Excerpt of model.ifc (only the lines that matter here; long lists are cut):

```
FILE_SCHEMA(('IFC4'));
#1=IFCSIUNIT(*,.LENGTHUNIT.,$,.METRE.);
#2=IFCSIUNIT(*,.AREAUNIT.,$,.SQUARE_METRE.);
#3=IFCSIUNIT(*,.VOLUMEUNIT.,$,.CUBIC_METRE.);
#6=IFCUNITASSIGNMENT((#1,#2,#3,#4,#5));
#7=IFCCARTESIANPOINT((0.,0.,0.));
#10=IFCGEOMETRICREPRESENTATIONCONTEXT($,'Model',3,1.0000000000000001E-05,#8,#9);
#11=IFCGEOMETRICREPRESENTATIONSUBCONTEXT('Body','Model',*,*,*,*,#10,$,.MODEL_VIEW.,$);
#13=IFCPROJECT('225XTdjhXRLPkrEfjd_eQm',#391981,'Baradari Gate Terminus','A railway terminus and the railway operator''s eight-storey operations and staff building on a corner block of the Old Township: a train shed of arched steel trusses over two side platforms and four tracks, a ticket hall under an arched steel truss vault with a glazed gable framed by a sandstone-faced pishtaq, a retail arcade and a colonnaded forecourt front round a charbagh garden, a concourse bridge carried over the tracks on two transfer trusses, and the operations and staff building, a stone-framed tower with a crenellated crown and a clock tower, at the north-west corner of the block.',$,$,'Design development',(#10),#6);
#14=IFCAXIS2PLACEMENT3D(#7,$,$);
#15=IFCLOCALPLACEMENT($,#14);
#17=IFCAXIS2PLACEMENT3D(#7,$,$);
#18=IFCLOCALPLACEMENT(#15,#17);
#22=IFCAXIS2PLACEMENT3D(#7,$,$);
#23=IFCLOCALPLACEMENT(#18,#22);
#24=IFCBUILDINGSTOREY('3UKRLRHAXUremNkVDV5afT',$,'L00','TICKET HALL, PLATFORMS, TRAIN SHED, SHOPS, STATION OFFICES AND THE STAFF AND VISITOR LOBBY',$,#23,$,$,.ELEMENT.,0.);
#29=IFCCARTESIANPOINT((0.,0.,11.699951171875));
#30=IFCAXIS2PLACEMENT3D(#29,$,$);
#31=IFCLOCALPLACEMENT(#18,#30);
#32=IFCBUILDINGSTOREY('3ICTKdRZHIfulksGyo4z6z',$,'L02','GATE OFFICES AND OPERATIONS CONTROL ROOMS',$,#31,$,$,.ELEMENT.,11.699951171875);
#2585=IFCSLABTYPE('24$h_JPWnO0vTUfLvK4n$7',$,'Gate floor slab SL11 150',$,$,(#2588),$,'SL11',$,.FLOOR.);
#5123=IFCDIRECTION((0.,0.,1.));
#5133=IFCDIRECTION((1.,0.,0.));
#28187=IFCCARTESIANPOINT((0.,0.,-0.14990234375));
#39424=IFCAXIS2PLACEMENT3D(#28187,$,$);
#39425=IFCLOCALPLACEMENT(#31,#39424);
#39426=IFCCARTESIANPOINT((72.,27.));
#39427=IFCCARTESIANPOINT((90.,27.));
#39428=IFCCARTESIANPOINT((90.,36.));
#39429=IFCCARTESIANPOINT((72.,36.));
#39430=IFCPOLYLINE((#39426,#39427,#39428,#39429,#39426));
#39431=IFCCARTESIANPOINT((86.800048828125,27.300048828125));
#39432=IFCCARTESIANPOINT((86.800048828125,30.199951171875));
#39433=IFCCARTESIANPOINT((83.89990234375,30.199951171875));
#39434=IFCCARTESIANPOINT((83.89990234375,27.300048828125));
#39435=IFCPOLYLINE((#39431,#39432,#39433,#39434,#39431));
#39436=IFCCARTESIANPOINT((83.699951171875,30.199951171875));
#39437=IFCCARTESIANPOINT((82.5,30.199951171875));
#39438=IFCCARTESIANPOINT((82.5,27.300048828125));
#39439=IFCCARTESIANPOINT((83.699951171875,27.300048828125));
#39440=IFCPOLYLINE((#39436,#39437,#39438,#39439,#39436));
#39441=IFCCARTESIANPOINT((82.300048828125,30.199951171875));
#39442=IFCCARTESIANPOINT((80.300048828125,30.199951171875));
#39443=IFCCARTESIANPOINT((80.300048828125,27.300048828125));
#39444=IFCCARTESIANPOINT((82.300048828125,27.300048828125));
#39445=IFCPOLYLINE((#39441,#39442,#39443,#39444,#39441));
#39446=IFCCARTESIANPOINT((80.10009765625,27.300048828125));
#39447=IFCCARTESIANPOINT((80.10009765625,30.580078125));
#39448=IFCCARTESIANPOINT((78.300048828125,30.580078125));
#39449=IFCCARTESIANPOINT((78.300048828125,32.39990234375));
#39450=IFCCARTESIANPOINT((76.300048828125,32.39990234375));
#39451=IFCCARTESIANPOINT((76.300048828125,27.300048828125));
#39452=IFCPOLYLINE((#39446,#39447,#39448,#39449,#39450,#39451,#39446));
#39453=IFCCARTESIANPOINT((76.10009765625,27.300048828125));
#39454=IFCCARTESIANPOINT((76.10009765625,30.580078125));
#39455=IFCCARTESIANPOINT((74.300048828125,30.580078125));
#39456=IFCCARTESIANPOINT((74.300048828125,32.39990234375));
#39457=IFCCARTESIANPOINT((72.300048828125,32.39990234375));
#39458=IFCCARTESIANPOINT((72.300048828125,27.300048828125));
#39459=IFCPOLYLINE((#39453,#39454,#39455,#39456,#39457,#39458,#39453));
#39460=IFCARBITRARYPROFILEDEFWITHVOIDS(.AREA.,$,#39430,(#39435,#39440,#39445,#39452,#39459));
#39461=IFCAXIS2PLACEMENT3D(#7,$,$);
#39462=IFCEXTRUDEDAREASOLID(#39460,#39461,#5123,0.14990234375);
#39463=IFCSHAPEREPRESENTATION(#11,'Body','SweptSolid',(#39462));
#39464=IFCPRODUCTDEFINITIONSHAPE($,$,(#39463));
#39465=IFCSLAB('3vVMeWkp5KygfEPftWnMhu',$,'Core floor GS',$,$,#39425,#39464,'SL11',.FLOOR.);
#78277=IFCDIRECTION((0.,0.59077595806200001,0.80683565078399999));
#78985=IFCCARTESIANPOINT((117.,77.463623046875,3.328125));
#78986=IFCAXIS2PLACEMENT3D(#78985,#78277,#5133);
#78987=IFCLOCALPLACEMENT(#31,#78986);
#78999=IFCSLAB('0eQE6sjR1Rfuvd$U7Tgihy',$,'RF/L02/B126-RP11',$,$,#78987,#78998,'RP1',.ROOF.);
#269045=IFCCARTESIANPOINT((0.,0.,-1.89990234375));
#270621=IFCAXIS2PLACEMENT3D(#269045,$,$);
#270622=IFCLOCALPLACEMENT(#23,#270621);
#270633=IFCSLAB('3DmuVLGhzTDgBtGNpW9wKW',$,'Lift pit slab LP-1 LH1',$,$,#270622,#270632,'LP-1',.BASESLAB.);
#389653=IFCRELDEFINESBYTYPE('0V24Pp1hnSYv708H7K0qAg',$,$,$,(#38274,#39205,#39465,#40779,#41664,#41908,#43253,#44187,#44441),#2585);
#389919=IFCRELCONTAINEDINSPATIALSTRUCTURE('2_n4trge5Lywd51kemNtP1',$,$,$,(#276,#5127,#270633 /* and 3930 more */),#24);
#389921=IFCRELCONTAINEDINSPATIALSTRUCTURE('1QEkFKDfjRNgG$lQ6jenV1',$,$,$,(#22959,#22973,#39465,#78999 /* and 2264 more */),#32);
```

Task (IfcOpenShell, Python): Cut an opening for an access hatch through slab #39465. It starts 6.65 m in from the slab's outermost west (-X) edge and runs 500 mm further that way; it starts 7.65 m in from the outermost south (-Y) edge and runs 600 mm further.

```python
import numpy as np
import ifcopenshell
import ifcopenshell.api.feature
import ifcopenshell.api.geometry
import ifcopenshell.api.root
import ifcopenshell.geom
import ifcopenshell.util.placement
import ifcopenshell.util.representation
import ifcopenshell.util.shape
import ifcopenshell.util.unit

model = ifcopenshell.open("model.ifc")
unit_scale = ifcopenshell.util.unit.calculate_unit_scale(model)
settings = ifcopenshell.geom.settings()


def volume(element):
    """Net volume in cubic metres, openings subtracted."""
    shape = ifcopenshell.geom.create_shape(settings, element)
    return ifcopenshell.util.shape.get_volume(shape.geometry)


slab = model.by_guid("3vVMeWkp5KygfEPftWnMhu")
before = volume(slab)

# Extent in the slab's own axes, in metres. The edges named are its -X and -Y sides.
slab_shape = ifcopenshell.geom.create_shape(settings, slab)
vertices = ifcopenshell.util.shape.get_vertices(slab_shape.geometry)
x_min, y_min, bottom = vertices.min(axis=0)
top = vertices[:, 2].max()

opening = ifcopenshell.api.root.create_entity(model, ifc_class="IfcOpeningElement", name="Access hatch opening", predefined_type="OPENING")
context = ifcopenshell.util.representation.get_context(model, "Model", "Body", "MODEL_VIEW")
width, depth = 0.5, 0.6
outline = [(0.0, 0.0), (width, 0.0), (width, depth), (0.0, depth), (0.0, 0.0)]
# Overshoot both faces by 50 mm so the cut is clean.
shape = ifcopenshell.api.geometry.add_slab_representation(
    model, context=context, depth=top - bottom + 0.1, polyline=outline
)
ifcopenshell.api.geometry.assign_representation(model, product=opening, representation=shape)

matrix = ifcopenshell.util.placement.get_local_placement(slab.ObjectPlacement)
matrix[:, 3] = matrix @ np.append(np.array([x_min + 6.65, y_min + 7.65, bottom - 0.05]) / unit_scale, 1.0)
ifcopenshell.api.geometry.edit_object_placement(model, product=opening, matrix=matrix, is_si=False)
ifcopenshell.api.feature.add_feature(model, feature=opening, element=slab)

after = volume(slab)

print(f"slab volume {before:.3f} -> {after:.3f} m3")

model.write("model_edited.ifc")
```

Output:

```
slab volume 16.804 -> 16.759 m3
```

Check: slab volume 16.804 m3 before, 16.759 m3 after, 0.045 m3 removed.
